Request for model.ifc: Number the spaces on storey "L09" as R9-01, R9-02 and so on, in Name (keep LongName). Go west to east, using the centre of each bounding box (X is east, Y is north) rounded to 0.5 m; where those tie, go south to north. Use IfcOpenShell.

First a look at what the model holds.

```python
import ifcopenshell
import ifcopenshell.util.element
import ifcopenshell.util.placement

model = ifcopenshell.open("model.ifc")
print(model.schema)
storey = next(s for s in model.by_type("IfcBuildingStorey") if s.Name == "L09")
spaces = [e for e in ifcopenshell.util.element.get_decomposition(storey) if e.is_a("IfcSpace")]
for e in sorted(spaces, key=lambda e: e.id()):
    origin = ifcopenshell.util.placement.get_local_placement(e.ObjectPlacement)[:3, 3]
    print(e.id(), e.Name, e.LongName, origin.round(2) + 0.0, sep=" | ")
```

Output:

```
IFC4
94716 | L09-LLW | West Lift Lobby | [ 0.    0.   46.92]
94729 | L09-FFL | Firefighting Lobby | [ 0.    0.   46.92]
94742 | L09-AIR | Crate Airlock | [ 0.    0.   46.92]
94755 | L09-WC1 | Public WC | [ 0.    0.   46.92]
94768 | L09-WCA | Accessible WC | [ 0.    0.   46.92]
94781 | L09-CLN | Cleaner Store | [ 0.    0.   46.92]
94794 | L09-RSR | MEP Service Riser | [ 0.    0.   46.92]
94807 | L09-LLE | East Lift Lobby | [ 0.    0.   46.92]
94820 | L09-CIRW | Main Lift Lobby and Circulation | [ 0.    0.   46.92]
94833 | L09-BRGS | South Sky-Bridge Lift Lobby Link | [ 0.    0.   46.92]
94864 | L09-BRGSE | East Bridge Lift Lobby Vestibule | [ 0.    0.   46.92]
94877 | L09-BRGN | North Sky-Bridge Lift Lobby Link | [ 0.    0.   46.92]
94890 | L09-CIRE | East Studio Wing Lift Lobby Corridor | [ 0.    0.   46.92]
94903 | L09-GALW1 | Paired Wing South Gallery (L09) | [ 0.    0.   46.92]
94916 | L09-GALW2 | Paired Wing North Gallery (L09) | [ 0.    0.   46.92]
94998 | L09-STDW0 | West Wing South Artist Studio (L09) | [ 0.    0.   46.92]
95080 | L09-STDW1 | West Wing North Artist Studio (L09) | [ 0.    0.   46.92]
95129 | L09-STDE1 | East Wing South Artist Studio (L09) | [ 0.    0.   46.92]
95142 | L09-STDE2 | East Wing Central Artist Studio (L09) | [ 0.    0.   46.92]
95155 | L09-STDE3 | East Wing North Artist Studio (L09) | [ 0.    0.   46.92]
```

```python
import ifcopenshell
import ifcopenshell.geom
import ifcopenshell.util.element
import ifcopenshell.util.shape

model = ifcopenshell.open("model.ifc")
settings = ifcopenshell.geom.settings()
settings.set("use-world-coords", True)


def centre(element):
    shape = ifcopenshell.geom.create_shape(settings, element)
    return ifcopenshell.util.shape.get_bbox_centroid(shape.geometry)


storey = next(s for s in model.by_type("IfcBuildingStorey") if s.Name == "L09")
spaces = [e for e in ifcopenshell.util.element.get_decomposition(storey) if e.is_a("IfcSpace")]

# Insertion points can sit at a corner or the storey origin, so sort by the geometry (in metres).
centres = {e: centre(e) for e in spaces}
spaces.sort(key=lambda e: (round(centres[e][0] / 0.5), centres[e][1]))

for i, e in enumerate(spaces, start=1):
    number = f"R9-{i:02d}"
    e.Name = number
    print(e.id(), number)

model.write("model_updated.ifc")
```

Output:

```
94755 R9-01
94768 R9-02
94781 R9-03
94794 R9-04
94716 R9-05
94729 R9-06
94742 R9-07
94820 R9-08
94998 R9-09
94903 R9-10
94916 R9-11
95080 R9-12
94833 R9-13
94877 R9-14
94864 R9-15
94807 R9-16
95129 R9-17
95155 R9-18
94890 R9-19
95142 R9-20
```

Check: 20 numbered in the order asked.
